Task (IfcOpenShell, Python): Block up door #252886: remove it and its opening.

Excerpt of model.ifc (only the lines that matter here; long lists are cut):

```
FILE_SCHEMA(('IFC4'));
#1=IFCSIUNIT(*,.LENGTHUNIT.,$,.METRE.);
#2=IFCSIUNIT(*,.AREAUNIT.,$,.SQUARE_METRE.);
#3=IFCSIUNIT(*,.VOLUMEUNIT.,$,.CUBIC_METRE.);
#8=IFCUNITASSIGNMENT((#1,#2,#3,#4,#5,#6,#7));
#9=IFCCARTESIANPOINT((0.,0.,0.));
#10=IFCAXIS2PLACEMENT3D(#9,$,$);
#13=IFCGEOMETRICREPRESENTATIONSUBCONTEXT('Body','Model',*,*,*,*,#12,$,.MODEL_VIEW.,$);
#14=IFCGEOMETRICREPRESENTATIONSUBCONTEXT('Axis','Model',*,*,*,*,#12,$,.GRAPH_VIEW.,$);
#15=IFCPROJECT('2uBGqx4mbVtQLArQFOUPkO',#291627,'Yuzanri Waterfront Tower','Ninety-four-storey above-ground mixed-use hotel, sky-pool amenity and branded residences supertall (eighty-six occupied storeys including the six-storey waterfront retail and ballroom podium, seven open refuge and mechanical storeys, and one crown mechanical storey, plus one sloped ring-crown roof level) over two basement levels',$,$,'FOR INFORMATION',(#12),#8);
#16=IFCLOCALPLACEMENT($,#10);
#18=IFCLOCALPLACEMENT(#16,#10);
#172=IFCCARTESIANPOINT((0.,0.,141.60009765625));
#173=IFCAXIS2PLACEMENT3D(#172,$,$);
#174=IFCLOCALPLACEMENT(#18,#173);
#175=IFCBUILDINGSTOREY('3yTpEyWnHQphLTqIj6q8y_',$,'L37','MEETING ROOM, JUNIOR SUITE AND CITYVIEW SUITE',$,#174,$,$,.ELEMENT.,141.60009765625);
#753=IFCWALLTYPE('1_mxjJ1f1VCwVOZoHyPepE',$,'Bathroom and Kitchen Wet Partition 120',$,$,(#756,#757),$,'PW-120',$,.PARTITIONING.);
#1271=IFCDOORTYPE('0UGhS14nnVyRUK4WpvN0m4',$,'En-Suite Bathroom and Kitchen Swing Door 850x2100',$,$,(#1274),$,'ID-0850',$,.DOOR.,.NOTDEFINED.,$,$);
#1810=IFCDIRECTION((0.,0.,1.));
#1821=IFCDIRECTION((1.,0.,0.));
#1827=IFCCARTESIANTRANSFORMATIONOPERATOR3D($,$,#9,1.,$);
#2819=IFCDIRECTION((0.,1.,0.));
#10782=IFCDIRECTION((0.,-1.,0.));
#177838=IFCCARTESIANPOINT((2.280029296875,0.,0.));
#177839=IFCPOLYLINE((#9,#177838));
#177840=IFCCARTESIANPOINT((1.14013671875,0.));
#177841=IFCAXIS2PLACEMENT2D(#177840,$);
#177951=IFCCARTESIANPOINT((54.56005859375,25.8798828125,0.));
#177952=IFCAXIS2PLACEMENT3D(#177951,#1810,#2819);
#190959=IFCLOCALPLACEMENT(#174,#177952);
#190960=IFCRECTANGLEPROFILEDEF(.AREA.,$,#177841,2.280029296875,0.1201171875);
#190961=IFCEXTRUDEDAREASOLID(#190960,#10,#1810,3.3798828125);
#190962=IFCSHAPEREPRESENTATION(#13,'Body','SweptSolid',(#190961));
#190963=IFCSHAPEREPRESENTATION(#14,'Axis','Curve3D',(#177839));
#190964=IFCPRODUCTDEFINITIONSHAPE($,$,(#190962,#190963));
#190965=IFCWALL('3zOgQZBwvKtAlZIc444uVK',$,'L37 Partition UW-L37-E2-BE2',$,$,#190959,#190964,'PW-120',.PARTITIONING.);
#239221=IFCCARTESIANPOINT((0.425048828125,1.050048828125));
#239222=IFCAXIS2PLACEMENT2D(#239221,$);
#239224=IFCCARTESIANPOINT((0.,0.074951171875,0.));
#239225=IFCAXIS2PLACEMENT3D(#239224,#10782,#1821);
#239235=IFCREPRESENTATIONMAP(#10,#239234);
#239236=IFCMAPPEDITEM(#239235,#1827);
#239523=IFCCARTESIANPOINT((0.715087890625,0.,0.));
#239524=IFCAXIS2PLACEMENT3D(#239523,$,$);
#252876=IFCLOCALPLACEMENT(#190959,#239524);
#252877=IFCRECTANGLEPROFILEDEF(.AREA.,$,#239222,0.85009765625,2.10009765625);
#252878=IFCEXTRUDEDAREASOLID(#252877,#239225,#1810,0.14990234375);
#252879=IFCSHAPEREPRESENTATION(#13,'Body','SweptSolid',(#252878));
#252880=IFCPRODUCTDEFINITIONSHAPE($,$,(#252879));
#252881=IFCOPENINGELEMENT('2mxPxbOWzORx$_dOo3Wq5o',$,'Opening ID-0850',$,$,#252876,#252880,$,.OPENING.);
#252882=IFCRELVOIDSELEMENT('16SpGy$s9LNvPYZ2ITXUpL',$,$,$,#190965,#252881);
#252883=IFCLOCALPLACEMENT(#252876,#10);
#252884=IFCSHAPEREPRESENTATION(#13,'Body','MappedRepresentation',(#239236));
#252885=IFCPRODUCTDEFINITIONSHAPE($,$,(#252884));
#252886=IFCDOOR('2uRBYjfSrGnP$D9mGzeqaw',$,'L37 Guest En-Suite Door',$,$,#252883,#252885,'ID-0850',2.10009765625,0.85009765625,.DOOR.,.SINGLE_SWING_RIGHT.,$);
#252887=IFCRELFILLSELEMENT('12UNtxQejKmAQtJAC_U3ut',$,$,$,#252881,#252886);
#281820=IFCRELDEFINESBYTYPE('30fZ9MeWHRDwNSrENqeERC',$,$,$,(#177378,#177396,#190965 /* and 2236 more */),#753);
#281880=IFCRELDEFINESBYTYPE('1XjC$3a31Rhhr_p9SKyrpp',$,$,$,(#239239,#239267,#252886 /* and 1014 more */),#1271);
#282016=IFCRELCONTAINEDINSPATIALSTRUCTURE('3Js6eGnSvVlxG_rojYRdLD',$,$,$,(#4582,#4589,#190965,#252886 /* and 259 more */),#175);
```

```python
import ifcopenshell
import ifcopenshell.api.feature
import ifcopenshell.api.root
import ifcopenshell.geom
import ifcopenshell.util.shape

model = ifcopenshell.open("model.ifc")
settings = ifcopenshell.geom.settings()


def volume(element):
    """Net volume in cubic metres, openings subtracted."""
    shape = ifcopenshell.geom.create_shape(settings, element)
    return ifcopenshell.util.shape.get_volume(shape.geometry)


door = model.by_guid("2uRBYjfSrGnP$D9mGzeqaw")
opening = door.FillsVoids[0].RelatingOpeningElement
wall = opening.VoidsElements[0].RelatingBuildingElement
before = volume(wall)

ifcopenshell.api.root.remove_product(model, product=door)
ifcopenshell.api.feature.remove_feature(model, feature=opening)

after = volume(wall)

print(f"wall volume {before:.3f} -> {after:.3f} m3")

model.write("model_v2.ifc")
```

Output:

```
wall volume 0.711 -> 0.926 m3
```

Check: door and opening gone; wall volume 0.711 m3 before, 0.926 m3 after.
